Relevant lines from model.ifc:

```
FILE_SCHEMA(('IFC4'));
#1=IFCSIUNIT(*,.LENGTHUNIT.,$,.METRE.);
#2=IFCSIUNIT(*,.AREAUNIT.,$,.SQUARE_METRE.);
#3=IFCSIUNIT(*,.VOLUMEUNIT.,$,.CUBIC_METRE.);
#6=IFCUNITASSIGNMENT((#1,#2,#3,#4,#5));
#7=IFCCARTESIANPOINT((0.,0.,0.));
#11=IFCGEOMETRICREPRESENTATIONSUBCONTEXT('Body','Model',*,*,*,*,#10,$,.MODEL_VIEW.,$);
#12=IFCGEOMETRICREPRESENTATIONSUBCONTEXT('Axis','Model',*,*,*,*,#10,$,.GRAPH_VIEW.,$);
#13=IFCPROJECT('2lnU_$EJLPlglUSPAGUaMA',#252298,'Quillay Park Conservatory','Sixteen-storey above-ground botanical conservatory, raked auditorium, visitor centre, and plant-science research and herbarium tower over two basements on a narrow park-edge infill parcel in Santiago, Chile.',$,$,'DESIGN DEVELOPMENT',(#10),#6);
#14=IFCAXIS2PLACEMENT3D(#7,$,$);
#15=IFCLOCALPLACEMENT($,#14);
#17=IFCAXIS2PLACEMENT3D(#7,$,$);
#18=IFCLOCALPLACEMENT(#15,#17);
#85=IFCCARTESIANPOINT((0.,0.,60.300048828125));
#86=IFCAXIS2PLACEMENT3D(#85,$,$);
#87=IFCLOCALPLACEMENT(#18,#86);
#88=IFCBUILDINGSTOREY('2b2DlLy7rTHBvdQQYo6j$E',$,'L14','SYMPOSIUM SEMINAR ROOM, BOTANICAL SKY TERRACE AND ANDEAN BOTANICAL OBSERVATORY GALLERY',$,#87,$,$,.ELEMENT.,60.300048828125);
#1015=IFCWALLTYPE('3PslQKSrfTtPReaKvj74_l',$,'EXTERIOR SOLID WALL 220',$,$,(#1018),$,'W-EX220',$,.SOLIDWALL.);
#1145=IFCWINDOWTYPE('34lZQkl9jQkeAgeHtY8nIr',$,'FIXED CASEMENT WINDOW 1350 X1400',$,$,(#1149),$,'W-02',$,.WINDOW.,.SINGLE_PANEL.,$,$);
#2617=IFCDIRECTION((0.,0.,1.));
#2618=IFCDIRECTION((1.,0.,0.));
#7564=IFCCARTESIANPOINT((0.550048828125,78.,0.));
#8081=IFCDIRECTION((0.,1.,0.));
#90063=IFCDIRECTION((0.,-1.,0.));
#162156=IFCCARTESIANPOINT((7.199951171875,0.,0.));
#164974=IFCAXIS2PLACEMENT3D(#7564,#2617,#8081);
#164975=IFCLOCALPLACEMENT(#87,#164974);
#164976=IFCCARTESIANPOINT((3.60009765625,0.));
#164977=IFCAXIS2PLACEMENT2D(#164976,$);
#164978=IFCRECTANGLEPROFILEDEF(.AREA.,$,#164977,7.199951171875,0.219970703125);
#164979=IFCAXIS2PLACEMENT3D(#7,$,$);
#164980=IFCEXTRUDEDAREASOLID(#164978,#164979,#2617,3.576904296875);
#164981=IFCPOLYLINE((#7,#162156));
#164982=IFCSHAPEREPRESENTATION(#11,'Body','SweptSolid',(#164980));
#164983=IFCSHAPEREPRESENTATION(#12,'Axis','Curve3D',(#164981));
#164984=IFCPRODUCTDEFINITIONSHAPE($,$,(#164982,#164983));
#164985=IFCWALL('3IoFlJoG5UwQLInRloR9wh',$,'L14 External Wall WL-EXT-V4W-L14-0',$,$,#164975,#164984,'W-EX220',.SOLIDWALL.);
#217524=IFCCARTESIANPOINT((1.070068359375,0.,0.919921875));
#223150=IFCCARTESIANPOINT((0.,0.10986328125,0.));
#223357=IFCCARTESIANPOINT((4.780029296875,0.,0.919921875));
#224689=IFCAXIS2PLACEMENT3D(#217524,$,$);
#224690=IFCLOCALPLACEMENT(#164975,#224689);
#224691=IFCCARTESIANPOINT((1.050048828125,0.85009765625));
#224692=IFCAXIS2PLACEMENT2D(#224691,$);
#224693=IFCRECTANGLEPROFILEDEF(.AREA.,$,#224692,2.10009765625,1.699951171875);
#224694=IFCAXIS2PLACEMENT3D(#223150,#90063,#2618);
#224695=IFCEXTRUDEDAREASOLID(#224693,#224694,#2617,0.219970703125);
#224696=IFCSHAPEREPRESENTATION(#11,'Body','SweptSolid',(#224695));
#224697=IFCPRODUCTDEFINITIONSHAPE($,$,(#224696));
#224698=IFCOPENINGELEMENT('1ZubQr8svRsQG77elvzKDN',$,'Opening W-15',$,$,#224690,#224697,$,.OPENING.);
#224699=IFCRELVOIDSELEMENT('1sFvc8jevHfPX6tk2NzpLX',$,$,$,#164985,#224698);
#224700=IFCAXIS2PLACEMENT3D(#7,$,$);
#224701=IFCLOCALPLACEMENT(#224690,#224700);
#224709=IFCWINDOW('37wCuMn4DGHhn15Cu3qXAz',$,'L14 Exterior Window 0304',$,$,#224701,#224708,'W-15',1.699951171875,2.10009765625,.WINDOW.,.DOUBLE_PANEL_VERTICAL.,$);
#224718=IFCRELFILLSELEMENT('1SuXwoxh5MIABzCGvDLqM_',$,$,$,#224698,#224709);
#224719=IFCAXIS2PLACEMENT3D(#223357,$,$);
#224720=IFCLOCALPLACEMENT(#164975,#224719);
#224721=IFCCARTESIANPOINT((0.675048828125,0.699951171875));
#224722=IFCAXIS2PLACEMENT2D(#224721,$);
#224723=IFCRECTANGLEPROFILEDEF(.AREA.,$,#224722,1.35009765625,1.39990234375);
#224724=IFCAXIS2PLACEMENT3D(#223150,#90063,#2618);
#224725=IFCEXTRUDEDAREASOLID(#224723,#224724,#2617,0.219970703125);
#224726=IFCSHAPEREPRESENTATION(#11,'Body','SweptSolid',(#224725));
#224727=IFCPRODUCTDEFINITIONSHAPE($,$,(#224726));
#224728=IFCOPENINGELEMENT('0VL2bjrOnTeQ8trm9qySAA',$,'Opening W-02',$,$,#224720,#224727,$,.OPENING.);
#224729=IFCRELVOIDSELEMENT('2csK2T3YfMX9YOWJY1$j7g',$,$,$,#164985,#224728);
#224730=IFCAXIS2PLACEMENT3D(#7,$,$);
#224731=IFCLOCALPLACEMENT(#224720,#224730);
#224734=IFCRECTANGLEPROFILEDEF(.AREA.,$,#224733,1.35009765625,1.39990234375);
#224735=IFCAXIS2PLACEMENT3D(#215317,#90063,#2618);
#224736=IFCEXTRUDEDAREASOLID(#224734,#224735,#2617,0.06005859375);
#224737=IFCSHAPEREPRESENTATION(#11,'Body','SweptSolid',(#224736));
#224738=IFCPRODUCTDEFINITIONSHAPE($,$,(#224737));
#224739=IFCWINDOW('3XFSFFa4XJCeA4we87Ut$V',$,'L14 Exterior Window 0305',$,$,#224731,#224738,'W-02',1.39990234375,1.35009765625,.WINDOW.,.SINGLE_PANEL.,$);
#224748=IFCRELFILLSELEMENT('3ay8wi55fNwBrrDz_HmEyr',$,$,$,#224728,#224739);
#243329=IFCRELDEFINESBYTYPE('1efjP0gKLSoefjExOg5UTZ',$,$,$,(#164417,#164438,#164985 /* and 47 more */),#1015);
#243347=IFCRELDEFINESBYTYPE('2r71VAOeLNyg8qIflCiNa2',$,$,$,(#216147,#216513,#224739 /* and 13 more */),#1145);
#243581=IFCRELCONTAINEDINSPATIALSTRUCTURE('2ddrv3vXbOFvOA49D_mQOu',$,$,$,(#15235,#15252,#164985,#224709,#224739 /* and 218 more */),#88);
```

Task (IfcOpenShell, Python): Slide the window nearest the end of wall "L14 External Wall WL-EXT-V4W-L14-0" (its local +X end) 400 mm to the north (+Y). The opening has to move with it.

```python
import ifcopenshell
import ifcopenshell.api.geometry
import ifcopenshell.util.placement
import ifcopenshell.util.unit

model = ifcopenshell.open("model.ifc")
unit_scale = ifcopenshell.util.unit.calculate_unit_scale(model)

window = model.by_guid("3XFSFFa4XJCeA4we87Ut$V")
opening = window.FillsVoids[0].RelatingOpeningElement
wall = opening.VoidsElements[0].RelatingBuildingElement

wall_matrix = ifcopenshell.util.placement.get_local_placement(wall.ObjectPlacement)
shift = wall_matrix[:3, 0] * 0.4 / unit_scale
before = ifcopenshell.util.placement.get_local_placement(window.ObjectPlacement)[:3, 3].copy()

# The window is placed relative to its opening, so it follows when the opening moves.
matrix = ifcopenshell.util.placement.get_local_placement(opening.ObjectPlacement)
matrix[:3, 3] += shift
ifcopenshell.api.geometry.edit_object_placement(
    model, product=opening, matrix=matrix, is_si=False, should_transform_children=True
)

after = ifcopenshell.util.placement.get_local_placement(window.ObjectPlacement)[:3, 3]
print("window moved by", (after - before).round(3) + 0.0)

model.write("model_v2.ifc")
```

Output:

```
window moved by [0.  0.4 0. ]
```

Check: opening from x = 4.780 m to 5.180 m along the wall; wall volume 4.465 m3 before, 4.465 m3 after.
